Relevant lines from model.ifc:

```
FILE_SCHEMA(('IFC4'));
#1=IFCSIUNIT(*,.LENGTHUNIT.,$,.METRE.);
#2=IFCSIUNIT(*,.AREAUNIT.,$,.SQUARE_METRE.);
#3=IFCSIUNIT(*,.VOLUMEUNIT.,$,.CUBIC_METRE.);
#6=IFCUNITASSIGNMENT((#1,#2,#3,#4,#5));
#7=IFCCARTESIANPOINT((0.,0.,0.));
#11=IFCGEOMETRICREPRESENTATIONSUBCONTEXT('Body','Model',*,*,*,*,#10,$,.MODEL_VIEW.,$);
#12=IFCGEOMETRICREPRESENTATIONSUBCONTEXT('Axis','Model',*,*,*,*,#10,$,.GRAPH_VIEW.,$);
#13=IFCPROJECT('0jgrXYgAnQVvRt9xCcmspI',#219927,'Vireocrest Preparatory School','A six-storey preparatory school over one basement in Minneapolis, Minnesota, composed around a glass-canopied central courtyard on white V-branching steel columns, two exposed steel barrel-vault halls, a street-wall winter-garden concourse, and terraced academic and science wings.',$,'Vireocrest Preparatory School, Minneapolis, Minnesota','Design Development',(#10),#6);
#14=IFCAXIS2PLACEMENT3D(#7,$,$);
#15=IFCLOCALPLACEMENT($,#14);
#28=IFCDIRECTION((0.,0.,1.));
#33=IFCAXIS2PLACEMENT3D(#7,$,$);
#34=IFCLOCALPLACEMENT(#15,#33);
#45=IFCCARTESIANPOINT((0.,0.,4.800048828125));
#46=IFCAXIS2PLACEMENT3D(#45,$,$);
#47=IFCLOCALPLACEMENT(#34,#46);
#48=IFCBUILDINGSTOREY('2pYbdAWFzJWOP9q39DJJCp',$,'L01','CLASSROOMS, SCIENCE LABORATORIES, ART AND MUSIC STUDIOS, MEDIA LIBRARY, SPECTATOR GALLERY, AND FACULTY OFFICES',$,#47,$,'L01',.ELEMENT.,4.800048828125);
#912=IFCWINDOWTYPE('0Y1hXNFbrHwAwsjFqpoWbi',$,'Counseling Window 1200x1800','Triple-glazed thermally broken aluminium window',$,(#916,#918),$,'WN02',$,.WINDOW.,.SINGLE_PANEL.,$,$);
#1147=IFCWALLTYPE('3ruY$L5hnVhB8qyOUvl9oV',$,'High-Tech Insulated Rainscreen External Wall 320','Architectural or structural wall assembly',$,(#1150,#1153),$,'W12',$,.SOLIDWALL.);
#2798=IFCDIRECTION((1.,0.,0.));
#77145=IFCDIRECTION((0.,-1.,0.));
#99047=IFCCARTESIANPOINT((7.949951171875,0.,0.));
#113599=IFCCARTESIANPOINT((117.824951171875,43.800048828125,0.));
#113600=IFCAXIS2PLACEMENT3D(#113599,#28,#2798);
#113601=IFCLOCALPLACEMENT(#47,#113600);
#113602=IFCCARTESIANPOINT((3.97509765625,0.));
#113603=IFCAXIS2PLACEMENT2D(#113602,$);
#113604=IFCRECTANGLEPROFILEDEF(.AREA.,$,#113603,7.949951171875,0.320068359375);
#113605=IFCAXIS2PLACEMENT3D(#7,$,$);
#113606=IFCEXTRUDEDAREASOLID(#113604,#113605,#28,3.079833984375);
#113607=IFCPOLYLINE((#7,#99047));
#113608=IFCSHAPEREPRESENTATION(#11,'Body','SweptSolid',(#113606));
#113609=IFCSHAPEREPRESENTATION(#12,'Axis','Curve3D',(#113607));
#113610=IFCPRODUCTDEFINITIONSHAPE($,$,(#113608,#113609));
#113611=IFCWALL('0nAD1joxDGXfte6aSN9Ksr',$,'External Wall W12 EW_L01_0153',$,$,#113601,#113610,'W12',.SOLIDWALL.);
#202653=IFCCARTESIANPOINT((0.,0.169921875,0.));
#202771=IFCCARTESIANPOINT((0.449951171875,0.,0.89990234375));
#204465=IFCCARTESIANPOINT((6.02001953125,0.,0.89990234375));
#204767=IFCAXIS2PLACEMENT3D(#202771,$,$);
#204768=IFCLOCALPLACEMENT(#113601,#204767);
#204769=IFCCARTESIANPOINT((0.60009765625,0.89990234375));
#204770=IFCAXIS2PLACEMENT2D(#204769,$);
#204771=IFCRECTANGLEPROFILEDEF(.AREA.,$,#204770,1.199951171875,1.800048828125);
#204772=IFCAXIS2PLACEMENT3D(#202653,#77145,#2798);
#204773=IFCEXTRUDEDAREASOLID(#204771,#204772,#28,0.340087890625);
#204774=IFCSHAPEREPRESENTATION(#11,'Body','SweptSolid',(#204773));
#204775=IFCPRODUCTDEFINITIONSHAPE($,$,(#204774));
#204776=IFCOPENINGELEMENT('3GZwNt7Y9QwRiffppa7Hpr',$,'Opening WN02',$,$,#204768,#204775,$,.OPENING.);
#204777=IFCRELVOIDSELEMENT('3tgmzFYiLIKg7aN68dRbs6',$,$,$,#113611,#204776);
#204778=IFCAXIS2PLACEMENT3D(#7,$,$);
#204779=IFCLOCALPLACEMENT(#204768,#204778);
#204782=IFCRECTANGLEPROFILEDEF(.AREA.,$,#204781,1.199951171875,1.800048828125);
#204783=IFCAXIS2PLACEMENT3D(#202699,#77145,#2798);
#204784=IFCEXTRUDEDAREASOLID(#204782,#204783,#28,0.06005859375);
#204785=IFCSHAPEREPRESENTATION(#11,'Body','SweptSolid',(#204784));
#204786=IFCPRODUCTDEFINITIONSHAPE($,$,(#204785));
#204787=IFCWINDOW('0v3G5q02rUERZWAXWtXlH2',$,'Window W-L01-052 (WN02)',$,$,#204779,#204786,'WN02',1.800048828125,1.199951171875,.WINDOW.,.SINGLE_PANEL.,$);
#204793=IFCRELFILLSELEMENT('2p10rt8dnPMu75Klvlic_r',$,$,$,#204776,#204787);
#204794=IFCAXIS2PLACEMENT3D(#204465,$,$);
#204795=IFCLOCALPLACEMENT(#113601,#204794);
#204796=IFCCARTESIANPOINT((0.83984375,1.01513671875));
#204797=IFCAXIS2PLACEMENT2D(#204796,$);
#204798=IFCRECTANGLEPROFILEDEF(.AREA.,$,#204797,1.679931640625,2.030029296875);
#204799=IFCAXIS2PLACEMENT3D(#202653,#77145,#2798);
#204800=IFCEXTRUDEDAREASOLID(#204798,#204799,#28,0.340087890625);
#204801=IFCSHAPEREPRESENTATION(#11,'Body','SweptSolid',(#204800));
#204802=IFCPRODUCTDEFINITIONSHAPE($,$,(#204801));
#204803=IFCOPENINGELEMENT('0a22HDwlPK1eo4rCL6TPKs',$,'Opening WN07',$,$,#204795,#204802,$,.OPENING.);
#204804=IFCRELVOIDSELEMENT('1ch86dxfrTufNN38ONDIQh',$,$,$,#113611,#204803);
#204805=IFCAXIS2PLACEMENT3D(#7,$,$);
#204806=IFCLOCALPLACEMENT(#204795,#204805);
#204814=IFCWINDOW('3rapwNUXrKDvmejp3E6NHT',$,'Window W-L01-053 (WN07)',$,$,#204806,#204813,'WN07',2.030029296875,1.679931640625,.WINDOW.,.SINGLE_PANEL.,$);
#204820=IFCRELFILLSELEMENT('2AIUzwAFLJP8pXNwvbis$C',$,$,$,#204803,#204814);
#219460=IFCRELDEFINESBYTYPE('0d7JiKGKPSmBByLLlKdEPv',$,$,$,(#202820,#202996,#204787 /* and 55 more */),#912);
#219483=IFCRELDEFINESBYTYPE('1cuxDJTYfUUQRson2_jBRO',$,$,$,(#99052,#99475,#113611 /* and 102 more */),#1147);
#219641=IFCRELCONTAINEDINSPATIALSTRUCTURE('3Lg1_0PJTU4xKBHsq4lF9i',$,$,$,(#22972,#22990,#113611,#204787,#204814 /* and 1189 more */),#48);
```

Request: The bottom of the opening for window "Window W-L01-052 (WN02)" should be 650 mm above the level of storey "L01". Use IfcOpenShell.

```python
import numpy as np
import ifcopenshell
import ifcopenshell.api.geometry
import ifcopenshell.geom
import ifcopenshell.util.element
import ifcopenshell.util.placement
import ifcopenshell.util.shape
import ifcopenshell.util.unit

model = ifcopenshell.open("model.ifc")
unit_scale = ifcopenshell.util.unit.calculate_unit_scale(model)

window = model.by_guid("0v3G5q02rUERZWAXWtXlH2")
opening = window.FillsVoids[0].RelatingOpeningElement
storey = ifcopenshell.util.element.get_container(window, ifc_class="IfcBuildingStorey")
level = ifcopenshell.util.placement.get_local_placement(storey.ObjectPlacement)[2, 3]

# The opening's origin need not be at the sill, so measure its lowest point.
shape = ifcopenshell.geom.create_shape(ifcopenshell.geom.settings(), opening)
bottom = ifcopenshell.util.shape.get_shape_bottom_elevation(shape, shape.geometry) / unit_scale
dz = level + 0.65 / unit_scale - bottom

shift = np.array([0.0, 0.0, dz])
# The window is placed relative to its opening, so it follows when the opening moves.
matrix = ifcopenshell.util.placement.get_local_placement(opening.ObjectPlacement)
matrix[:3, 3] += shift
ifcopenshell.api.geometry.edit_object_placement(
    model, product=opening, matrix=matrix, is_si=False, should_transform_children=True
)

print(f"moved by {dz * unit_scale:+.3f} m")

model.write("model_v2.ifc")
```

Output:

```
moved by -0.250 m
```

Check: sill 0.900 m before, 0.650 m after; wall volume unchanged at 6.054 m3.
